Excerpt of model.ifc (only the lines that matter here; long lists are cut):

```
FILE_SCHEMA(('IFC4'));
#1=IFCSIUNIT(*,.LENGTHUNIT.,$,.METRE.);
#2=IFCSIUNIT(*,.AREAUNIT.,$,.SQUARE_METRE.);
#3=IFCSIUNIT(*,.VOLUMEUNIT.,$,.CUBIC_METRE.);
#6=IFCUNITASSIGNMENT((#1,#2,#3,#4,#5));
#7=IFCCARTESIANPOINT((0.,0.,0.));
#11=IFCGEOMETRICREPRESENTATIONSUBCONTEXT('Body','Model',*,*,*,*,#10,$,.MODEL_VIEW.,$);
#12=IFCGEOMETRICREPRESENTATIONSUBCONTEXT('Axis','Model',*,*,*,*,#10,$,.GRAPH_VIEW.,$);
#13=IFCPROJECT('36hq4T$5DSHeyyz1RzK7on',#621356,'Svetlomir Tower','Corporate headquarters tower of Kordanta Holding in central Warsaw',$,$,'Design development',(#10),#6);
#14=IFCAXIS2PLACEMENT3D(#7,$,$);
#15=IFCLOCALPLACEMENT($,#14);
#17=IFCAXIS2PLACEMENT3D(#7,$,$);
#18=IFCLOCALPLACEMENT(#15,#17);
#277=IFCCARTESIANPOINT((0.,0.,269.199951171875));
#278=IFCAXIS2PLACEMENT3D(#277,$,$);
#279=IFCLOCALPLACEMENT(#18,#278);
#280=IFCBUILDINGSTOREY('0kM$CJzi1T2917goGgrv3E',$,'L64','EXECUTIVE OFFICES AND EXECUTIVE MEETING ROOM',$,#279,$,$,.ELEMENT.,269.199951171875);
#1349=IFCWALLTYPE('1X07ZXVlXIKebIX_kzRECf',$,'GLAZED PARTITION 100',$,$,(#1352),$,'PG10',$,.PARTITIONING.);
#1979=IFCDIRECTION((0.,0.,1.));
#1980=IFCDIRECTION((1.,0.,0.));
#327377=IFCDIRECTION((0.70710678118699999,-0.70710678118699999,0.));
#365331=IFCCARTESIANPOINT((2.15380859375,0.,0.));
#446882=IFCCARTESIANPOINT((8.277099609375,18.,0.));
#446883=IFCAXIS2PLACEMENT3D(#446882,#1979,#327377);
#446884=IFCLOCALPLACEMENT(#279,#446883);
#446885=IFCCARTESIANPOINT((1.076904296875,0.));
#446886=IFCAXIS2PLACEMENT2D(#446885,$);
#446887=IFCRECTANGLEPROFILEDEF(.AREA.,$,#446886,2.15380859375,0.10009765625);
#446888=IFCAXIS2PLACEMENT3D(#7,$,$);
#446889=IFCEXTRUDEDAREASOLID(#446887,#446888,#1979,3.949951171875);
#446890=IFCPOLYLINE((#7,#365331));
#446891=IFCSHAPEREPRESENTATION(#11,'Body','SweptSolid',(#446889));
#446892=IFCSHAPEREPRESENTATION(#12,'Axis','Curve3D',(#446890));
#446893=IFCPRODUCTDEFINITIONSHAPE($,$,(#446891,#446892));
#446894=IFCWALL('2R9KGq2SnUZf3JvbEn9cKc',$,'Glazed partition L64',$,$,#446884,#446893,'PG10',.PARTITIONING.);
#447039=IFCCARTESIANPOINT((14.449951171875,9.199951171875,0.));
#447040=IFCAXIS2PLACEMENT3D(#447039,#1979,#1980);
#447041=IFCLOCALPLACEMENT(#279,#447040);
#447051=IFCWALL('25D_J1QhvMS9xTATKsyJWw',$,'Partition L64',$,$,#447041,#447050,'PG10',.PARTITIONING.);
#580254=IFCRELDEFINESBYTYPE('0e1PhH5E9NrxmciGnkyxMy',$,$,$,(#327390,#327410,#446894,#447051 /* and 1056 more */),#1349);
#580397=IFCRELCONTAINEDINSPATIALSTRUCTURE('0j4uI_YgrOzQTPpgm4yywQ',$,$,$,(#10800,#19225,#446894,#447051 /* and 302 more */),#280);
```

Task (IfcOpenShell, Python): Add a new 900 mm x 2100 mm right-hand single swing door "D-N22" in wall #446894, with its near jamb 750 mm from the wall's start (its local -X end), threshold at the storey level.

```python
import numpy as np
import ifcopenshell
import ifcopenshell.api.feature
import ifcopenshell.api.geometry
import ifcopenshell.api.root
import ifcopenshell.api.spatial
import ifcopenshell.geom
import ifcopenshell.util.element
import ifcopenshell.util.placement
import ifcopenshell.util.representation
import ifcopenshell.util.shape
import ifcopenshell.util.unit

model = ifcopenshell.open("model.ifc")
unit_scale = ifcopenshell.util.unit.calculate_unit_scale(model)
settings = ifcopenshell.geom.settings()


def volume(element):
    """Net volume in cubic metres, openings subtracted."""
    shape = ifcopenshell.geom.create_shape(settings, element)
    return ifcopenshell.util.shape.get_volume(shape.geometry)


wall = model.by_guid("2R9KGq2SnUZf3JvbEn9cKc")
storey = ifcopenshell.util.element.get_container(wall, ifc_class="IfcBuildingStorey")
context = ifcopenshell.util.representation.get_context(model, "Model", "Body", "MODEL_VIEW")
before = volume(wall)

width, height, from_end, sill = 0.9, 2.1, 0.75, 0.0  # metres

# The wall runs along its own X axis, and the end named is its -X end.
wall_shape = ifcopenshell.geom.create_shape(settings, wall)
x, y, z = ifcopenshell.util.shape.get_vertices(wall_shape.geometry).T
start = x.min() + from_end
face, thickness = float(y.min()), float(y.max() - y.min())
wall_matrix = ifcopenshell.util.placement.get_local_placement(wall.ObjectPlacement)
level = ifcopenshell.util.placement.get_local_placement(storey.ObjectPlacement)[2, 3]


def in_wall(x, y):
    """Placement at x, y metres in the wall's axes, at sill height."""
    matrix = wall_matrix.copy()
    matrix[:, 3] = wall_matrix @ np.array([x / unit_scale, y / unit_scale, 0.0, 1.0])
    matrix[2, 3] = level + sill / unit_scale
    return matrix


# Opening: a box that overshoots both wall faces by 50 mm.
opening = ifcopenshell.api.root.create_entity(model, ifc_class="IfcOpeningElement", predefined_type="OPENING")
box = ifcopenshell.api.geometry.add_wall_representation(
    model, context=context, length=width, height=height, thickness=thickness + 0.1
)
ifcopenshell.api.geometry.assign_representation(model, product=opening, representation=box)
ifcopenshell.api.geometry.edit_object_placement(model, product=opening, matrix=in_wall(start, face - 0.05), is_si=False)
ifcopenshell.api.feature.add_feature(model, feature=opening, element=wall)

door = ifcopenshell.api.root.create_entity(model, ifc_class="IfcDoor", name="D-N22", predefined_type="DOOR")
door.OverallWidth, door.OverallHeight = width / unit_scale, height / unit_scale
door.OperationType = "SINGLE_SWING_RIGHT"
body = ifcopenshell.api.geometry.add_door_representation(
    model,
    context=context,
    overall_width=door.OverallWidth,
    overall_height=door.OverallHeight,
    operation_type="SINGLE_SWING_RIGHT",
    lining_properties={"LiningDepth": thickness / unit_scale, "ThresholdDepth": thickness / unit_scale},
)
ifcopenshell.api.geometry.assign_representation(model, product=door, representation=body)
ifcopenshell.api.spatial.assign_container(model, products=[door], relating_structure=storey)
ifcopenshell.api.feature.add_filling(model, opening=opening, element=door)

# The lining spans the wall, so the door starts at the wall face.
ifcopenshell.api.geometry.edit_object_placement(model, product=door, matrix=in_wall(start, face), is_si=False)

after = volume(wall)

print(f"wall volume {before:.3f} -> {after:.3f} m3")

model.write("model-out.ifc")
```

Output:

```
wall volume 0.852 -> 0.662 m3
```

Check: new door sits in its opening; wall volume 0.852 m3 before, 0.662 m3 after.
